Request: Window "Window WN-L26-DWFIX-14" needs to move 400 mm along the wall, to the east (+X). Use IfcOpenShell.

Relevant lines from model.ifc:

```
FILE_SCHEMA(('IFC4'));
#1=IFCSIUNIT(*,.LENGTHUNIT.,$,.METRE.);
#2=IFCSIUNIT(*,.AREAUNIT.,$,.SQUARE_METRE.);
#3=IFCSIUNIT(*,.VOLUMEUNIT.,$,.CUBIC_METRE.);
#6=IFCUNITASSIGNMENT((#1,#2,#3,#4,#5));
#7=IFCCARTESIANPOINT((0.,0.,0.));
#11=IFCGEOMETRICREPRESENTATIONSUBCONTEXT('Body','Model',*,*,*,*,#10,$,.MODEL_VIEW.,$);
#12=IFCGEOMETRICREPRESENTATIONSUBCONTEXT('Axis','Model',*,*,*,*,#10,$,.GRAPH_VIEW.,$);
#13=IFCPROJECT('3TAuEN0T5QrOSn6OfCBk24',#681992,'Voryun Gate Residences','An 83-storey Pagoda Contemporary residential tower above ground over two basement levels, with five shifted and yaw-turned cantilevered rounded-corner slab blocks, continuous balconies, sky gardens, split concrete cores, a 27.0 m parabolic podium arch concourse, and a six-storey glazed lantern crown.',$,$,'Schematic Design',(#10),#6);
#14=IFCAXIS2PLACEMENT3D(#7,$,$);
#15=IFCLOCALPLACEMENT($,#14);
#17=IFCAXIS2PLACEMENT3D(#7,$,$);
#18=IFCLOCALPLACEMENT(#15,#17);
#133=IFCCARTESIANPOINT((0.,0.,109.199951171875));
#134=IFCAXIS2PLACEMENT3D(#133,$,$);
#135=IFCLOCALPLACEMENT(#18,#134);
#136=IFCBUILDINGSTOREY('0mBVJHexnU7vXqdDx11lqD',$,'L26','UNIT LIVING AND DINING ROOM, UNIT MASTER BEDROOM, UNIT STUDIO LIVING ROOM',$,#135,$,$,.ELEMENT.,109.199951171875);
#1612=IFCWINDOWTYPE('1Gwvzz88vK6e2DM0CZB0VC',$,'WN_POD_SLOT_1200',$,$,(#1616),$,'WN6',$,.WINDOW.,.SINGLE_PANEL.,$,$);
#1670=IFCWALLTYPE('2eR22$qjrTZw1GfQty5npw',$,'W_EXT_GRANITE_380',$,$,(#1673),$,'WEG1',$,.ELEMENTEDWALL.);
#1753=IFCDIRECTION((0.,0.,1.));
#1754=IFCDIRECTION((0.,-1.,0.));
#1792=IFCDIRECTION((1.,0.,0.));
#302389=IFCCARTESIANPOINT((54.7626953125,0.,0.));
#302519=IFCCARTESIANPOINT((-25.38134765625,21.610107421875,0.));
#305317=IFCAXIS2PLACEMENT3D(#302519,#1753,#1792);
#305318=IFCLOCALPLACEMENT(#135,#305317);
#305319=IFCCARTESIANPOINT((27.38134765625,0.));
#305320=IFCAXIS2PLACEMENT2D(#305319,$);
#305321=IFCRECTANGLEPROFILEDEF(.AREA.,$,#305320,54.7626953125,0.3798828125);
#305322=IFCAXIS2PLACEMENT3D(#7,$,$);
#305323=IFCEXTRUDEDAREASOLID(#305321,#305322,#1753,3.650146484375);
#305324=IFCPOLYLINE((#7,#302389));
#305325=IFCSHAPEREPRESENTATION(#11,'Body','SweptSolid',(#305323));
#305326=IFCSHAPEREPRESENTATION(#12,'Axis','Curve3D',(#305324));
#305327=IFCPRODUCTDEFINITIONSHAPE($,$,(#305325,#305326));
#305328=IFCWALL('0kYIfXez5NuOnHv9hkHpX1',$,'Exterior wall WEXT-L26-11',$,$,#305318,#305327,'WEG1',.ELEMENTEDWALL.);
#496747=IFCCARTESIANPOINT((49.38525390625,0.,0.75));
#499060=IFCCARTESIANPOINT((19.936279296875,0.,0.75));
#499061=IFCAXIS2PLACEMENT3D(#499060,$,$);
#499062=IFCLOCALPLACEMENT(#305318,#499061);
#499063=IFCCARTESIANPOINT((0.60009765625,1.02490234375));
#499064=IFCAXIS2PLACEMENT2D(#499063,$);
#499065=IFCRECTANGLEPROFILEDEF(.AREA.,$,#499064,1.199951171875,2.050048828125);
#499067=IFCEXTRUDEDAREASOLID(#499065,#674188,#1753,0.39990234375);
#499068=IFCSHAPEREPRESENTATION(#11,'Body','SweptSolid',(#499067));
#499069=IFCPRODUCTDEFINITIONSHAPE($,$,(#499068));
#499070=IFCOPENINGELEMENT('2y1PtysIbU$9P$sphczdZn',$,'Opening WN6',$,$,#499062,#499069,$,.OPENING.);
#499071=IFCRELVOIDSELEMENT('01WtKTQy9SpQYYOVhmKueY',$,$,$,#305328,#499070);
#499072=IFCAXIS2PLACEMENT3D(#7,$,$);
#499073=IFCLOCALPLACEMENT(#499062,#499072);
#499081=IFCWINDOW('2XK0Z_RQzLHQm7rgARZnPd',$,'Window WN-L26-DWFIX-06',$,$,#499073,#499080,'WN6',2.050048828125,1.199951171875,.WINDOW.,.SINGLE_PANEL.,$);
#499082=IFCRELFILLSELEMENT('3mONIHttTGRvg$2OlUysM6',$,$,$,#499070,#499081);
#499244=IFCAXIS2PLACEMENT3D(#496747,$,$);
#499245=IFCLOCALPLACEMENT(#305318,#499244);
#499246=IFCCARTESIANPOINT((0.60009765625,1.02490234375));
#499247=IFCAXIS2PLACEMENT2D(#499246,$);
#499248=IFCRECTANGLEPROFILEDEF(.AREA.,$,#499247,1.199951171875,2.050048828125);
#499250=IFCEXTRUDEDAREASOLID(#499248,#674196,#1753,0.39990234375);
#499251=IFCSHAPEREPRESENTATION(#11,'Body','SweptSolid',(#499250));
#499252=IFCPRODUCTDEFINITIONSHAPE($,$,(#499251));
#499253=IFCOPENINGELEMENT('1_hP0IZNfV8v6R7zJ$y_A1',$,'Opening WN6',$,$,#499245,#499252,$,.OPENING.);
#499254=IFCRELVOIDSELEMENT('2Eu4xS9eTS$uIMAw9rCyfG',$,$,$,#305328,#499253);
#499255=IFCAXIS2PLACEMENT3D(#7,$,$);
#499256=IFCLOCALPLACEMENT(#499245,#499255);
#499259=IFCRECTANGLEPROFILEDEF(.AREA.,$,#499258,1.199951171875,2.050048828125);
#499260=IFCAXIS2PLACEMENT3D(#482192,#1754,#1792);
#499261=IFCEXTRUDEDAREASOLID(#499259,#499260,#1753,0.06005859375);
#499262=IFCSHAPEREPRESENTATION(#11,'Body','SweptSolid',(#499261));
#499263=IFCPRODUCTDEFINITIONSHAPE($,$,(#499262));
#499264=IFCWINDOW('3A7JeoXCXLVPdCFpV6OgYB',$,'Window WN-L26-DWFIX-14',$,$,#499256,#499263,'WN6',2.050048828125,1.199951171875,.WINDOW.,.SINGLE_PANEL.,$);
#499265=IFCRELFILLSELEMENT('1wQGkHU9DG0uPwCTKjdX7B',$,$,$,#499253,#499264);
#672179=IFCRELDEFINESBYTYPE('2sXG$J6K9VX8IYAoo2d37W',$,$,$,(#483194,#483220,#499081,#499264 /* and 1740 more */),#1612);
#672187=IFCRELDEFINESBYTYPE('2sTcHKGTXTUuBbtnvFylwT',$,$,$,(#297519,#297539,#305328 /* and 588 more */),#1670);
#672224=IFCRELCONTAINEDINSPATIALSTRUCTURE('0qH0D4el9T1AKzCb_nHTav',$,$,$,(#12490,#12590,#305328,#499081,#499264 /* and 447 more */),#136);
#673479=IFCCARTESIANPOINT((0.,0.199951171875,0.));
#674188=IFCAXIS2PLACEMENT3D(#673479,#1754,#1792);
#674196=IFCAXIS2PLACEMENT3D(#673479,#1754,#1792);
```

```python
import ifcopenshell
import ifcopenshell.api.geometry
import ifcopenshell.util.placement
import ifcopenshell.util.unit

model = ifcopenshell.open("model.ifc")
unit_scale = ifcopenshell.util.unit.calculate_unit_scale(model)

window = model.by_guid("3A7JeoXCXLVPdCFpV6OgYB")
opening = window.FillsVoids[0].RelatingOpeningElement
wall = opening.VoidsElements[0].RelatingBuildingElement

wall_matrix = ifcopenshell.util.placement.get_local_placement(wall.ObjectPlacement)
shift = wall_matrix[:3, 0] * 0.4 / unit_scale
before = ifcopenshell.util.placement.get_local_placement(window.ObjectPlacement)[:3, 3].copy()

# The window is placed relative to its opening, so it follows when the opening moves.
matrix = ifcopenshell.util.placement.get_local_placement(opening.ObjectPlacement)
matrix[:3, 3] += shift
ifcopenshell.api.geometry.edit_object_placement(
    model, product=opening, matrix=matrix, is_si=False, should_transform_children=True
)

after = ifcopenshell.util.placement.get_local_placement(window.ObjectPlacement)[:3, 3]
print("window moved by", (after - before).round(3) + 0.0)

model.write("model_updated.ifc")
```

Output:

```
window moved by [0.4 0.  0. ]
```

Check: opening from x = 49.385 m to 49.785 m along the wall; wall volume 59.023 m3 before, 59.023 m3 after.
